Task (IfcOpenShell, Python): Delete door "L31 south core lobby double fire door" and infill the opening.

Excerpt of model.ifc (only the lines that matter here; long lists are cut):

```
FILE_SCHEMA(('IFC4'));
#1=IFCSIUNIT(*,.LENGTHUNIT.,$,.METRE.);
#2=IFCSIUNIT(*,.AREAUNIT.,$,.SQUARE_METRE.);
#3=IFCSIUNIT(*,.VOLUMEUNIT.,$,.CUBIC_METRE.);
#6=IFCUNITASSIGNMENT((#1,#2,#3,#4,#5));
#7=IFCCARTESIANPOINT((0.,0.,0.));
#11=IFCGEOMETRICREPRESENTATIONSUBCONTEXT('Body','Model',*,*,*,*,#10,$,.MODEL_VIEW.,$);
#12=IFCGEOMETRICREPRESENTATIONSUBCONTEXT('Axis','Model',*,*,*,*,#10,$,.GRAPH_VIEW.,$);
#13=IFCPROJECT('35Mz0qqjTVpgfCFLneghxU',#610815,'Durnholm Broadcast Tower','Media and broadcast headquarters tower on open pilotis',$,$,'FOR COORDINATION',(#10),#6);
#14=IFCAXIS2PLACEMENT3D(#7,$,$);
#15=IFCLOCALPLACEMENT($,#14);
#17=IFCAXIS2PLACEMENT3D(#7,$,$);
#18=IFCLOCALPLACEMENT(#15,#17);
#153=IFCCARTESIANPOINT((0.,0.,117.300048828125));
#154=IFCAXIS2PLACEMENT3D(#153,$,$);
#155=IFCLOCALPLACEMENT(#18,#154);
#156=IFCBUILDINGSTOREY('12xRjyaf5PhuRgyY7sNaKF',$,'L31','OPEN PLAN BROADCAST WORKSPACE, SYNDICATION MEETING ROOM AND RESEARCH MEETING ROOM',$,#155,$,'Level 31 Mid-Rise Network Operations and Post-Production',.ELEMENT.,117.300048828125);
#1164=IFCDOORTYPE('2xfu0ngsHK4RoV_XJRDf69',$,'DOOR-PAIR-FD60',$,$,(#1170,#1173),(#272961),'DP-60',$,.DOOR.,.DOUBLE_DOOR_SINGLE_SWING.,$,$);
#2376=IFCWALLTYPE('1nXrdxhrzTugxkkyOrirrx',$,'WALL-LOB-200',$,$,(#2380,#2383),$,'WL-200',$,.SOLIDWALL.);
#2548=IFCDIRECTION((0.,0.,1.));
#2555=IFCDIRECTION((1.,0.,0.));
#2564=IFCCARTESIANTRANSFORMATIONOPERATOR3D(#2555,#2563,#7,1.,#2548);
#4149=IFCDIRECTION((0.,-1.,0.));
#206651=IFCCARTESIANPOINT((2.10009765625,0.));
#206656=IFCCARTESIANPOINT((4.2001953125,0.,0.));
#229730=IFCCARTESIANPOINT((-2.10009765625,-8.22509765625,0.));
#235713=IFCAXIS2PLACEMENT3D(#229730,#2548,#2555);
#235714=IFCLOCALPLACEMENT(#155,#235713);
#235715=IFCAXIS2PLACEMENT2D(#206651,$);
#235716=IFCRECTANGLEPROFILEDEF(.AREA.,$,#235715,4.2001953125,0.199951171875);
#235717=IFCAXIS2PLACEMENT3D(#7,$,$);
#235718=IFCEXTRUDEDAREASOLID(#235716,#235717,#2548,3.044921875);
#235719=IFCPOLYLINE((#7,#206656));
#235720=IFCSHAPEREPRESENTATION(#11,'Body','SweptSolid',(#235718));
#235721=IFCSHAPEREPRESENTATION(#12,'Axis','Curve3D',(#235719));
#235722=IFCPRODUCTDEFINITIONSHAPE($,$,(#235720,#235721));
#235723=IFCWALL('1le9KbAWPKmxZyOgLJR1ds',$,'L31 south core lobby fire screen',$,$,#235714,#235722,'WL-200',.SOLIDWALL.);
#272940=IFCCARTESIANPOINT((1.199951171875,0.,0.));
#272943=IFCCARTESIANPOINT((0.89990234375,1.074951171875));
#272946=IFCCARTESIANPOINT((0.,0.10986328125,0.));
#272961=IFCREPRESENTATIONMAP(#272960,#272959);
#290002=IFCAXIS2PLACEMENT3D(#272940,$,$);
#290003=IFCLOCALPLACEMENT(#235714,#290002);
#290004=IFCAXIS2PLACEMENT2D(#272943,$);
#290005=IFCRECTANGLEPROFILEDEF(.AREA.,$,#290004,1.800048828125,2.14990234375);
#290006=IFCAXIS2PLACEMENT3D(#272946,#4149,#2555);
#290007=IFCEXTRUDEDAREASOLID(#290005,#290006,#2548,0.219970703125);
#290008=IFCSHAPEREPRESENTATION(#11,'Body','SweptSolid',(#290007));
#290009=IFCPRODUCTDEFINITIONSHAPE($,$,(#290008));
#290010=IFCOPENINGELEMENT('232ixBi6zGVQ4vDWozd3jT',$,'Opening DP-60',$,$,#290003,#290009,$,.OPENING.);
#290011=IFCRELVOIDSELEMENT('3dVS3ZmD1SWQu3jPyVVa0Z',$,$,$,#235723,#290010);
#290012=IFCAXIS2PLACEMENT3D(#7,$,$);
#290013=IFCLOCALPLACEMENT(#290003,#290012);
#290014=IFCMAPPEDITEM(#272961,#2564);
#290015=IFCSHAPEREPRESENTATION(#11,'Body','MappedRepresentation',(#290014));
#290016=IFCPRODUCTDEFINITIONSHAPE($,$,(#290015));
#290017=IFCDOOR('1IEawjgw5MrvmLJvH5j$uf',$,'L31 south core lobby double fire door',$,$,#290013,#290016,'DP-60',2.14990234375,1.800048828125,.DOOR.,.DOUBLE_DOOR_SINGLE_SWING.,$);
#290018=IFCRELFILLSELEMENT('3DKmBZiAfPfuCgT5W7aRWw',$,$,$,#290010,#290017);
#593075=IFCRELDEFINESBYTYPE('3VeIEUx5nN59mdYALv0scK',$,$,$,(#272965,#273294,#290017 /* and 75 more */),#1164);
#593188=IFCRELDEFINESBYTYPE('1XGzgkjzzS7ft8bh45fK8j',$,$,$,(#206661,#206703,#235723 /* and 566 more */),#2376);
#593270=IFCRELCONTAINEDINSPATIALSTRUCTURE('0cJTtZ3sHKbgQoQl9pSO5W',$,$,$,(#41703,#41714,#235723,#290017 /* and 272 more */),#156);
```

```python
import ifcopenshell
import ifcopenshell.api.feature
import ifcopenshell.api.root
import ifcopenshell.geom
import ifcopenshell.util.shape

model = ifcopenshell.open("model.ifc")
settings = ifcopenshell.geom.settings()


def volume(element):
    """Net volume in cubic metres, openings subtracted."""
    shape = ifcopenshell.geom.create_shape(settings, element)
    return ifcopenshell.util.shape.get_volume(shape.geometry)


door = model.by_guid("1IEawjgw5MrvmLJvH5j$uf")
opening = door.FillsVoids[0].RelatingOpeningElement
wall = opening.VoidsElements[0].RelatingBuildingElement
before = volume(wall)

ifcopenshell.api.root.remove_product(model, product=door)
ifcopenshell.api.feature.remove_feature(model, feature=opening)

after = volume(wall)

print(f"wall volume {before:.3f} -> {after:.3f} m3")

model.write("model_updated.ifc")
```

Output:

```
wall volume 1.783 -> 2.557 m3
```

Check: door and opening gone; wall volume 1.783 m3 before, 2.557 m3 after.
